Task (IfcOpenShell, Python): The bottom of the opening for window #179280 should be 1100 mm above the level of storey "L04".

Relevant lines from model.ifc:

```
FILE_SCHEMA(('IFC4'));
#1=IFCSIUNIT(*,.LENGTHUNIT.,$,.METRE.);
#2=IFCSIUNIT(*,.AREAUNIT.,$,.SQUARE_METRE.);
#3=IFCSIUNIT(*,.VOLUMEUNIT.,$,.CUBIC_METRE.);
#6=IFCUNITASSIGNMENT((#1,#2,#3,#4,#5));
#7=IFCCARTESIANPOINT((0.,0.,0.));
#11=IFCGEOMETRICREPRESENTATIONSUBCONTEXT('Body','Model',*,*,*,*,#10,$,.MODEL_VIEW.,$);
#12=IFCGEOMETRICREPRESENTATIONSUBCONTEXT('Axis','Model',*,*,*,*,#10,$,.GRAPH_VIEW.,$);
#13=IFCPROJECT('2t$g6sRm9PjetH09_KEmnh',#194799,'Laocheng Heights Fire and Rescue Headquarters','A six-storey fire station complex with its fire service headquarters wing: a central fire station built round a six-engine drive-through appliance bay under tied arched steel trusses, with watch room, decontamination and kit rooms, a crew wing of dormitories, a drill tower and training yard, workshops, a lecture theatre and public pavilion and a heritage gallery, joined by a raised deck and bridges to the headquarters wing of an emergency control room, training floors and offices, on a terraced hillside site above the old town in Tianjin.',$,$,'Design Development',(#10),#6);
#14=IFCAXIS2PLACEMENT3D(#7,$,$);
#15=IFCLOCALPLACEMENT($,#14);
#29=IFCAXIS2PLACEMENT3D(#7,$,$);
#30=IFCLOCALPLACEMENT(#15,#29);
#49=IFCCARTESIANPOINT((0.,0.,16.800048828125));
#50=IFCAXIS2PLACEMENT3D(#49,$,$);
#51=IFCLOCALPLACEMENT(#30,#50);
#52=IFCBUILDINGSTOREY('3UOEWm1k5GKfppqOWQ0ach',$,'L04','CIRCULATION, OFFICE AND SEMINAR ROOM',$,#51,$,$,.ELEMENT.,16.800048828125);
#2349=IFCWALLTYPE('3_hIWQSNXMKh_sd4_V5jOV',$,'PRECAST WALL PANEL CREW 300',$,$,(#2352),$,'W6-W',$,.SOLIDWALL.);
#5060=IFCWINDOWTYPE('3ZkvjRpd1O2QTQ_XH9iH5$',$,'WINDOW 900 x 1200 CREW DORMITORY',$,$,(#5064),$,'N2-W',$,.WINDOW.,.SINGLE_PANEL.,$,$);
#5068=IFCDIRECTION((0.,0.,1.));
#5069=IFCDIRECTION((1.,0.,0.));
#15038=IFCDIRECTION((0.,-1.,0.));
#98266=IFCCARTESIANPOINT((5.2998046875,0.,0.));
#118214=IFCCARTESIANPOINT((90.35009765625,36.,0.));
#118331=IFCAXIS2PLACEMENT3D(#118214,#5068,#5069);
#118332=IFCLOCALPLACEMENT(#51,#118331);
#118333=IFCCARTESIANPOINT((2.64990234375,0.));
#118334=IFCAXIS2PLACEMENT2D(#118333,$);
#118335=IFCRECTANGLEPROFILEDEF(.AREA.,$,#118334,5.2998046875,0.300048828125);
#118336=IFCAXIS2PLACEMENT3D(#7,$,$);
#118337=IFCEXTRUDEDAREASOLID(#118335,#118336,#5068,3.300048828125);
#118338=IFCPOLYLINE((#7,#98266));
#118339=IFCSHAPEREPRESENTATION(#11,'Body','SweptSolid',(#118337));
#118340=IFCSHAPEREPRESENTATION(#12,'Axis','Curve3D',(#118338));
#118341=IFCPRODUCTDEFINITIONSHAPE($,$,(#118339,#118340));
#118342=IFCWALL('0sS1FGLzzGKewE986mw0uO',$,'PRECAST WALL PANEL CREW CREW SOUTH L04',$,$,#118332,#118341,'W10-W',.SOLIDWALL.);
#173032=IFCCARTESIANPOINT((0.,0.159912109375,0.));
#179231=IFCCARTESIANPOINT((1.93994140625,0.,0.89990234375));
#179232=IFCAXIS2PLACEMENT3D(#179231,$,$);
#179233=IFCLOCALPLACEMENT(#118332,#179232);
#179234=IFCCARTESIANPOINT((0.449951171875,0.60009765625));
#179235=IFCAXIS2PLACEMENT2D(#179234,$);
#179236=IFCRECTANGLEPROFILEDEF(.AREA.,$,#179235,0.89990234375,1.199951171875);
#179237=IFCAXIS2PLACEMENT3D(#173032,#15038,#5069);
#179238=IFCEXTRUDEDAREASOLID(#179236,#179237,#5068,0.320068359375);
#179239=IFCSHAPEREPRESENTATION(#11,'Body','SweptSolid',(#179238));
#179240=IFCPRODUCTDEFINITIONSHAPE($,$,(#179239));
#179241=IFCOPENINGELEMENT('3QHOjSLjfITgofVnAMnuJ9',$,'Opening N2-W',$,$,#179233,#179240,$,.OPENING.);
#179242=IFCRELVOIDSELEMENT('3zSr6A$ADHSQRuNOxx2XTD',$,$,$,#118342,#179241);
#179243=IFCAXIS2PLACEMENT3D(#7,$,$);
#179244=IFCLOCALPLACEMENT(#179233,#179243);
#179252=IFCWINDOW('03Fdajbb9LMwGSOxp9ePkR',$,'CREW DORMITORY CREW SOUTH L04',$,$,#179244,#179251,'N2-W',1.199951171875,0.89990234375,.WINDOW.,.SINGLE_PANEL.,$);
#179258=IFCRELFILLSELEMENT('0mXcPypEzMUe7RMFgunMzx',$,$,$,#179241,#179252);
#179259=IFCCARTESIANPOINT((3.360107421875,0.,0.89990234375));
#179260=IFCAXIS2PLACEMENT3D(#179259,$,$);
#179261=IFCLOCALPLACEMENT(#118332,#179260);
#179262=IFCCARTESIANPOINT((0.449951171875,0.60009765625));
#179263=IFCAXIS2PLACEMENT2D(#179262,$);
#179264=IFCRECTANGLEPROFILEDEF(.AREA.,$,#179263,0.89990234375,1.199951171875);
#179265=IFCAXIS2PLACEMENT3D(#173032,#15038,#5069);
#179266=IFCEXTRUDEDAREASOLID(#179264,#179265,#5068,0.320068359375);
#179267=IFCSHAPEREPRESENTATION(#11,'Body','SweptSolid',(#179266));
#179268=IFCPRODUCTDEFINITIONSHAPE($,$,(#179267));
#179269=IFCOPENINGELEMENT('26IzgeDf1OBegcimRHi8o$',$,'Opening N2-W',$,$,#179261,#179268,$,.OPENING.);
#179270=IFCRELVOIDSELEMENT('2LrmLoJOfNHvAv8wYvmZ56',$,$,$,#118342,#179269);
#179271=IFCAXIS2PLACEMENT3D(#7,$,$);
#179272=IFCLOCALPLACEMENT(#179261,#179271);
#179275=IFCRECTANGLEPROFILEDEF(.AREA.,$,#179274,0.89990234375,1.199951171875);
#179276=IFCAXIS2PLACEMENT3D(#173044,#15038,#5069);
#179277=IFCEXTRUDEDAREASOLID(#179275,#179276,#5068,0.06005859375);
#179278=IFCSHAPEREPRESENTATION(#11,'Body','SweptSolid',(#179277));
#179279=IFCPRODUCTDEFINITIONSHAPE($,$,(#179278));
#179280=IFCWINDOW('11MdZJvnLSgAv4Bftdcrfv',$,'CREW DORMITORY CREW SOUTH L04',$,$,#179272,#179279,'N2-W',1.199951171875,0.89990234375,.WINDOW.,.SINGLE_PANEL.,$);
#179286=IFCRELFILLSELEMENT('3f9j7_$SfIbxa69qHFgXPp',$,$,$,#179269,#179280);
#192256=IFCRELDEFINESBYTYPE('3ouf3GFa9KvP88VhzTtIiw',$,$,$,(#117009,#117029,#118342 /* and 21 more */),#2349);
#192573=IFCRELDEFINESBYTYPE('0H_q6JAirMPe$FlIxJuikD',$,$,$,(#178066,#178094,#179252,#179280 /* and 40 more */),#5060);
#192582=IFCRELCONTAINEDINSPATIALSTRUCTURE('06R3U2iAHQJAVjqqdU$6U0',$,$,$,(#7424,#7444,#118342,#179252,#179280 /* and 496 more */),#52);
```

```python
import numpy as np
import ifcopenshell
import ifcopenshell.api.geometry
import ifcopenshell.geom
import ifcopenshell.util.element
import ifcopenshell.util.placement
import ifcopenshell.util.shape
import ifcopenshell.util.unit

model = ifcopenshell.open("model.ifc")
unit_scale = ifcopenshell.util.unit.calculate_unit_scale(model)

window = model.by_id(179280)
opening = window.FillsVoids[0].RelatingOpeningElement
storey = ifcopenshell.util.element.get_container(window, ifc_class="IfcBuildingStorey")
level = ifcopenshell.util.placement.get_local_placement(storey.ObjectPlacement)[2, 3]

# The opening's origin need not be at the sill, so measure its lowest point.
shape = ifcopenshell.geom.create_shape(ifcopenshell.geom.settings(), opening)
bottom = ifcopenshell.util.shape.get_shape_bottom_elevation(shape, shape.geometry) / unit_scale
dz = level + 1.1 / unit_scale - bottom

shift = np.array([0.0, 0.0, dz])
# The window is placed relative to its opening, so it follows when the opening moves.
matrix = ifcopenshell.util.placement.get_local_placement(opening.ObjectPlacement)
matrix[:3, 3] += shift
ifcopenshell.api.geometry.edit_object_placement(
    model, product=opening, matrix=matrix, is_si=False, should_transform_children=True
)

print(f"moved by {dz * unit_scale:+.3f} m")

model.write("model-out.ifc")
```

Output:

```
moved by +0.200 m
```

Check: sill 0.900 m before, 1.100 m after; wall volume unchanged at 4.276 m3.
